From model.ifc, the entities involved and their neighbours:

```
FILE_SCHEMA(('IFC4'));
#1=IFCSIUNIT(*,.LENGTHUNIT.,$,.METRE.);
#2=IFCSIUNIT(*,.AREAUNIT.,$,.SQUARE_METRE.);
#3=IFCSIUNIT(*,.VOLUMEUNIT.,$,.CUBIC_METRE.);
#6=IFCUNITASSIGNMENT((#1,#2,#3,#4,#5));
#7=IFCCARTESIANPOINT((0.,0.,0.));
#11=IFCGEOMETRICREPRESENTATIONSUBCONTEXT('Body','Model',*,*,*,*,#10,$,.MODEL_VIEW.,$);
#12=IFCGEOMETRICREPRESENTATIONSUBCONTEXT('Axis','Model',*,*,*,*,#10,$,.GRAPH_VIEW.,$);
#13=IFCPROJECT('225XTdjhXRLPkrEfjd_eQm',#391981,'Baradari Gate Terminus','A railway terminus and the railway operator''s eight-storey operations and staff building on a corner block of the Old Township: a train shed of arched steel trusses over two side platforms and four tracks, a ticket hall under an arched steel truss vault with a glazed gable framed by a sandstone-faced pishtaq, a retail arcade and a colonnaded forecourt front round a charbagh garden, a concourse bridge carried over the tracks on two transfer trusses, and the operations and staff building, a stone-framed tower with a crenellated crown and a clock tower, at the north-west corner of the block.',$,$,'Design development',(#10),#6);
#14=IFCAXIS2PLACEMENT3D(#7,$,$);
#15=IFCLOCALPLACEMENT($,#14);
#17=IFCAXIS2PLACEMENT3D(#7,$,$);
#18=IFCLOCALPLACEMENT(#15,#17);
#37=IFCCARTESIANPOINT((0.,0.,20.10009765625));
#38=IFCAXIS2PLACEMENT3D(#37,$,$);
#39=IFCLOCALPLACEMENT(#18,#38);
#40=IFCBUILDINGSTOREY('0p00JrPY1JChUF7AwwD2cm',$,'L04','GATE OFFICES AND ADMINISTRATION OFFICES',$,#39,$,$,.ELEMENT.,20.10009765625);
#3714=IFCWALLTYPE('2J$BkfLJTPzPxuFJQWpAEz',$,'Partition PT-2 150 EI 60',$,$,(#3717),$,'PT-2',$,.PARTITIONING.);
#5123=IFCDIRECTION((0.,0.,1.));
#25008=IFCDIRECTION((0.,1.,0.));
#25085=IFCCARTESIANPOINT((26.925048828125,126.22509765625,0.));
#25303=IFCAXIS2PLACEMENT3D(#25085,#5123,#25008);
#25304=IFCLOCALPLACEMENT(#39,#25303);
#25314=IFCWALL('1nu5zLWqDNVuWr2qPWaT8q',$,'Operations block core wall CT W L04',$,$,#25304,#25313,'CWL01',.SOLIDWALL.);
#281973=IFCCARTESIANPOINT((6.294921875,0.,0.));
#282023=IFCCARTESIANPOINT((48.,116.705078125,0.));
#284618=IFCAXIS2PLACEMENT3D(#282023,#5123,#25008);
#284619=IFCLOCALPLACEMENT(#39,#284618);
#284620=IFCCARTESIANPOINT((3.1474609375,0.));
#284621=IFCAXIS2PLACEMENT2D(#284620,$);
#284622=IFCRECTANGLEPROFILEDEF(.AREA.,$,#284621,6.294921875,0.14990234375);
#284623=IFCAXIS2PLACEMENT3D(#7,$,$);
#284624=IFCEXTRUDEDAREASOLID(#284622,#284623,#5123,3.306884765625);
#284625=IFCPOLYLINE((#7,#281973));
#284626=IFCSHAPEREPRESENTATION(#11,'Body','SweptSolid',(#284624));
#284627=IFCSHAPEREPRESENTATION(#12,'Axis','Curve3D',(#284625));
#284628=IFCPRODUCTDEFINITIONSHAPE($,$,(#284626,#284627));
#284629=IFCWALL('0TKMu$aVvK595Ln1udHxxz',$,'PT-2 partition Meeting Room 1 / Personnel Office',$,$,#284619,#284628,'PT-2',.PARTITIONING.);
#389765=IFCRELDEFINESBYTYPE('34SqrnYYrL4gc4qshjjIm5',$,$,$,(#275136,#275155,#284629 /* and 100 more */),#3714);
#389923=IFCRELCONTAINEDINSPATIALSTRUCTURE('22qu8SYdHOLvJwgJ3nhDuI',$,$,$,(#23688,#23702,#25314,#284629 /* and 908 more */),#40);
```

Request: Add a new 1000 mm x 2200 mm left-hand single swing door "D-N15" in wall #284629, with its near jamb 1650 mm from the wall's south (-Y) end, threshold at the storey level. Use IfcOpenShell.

```python
import numpy as np
import ifcopenshell
import ifcopenshell.api.feature
import ifcopenshell.api.geometry
import ifcopenshell.api.root
import ifcopenshell.api.spatial
import ifcopenshell.geom
import ifcopenshell.util.element
import ifcopenshell.util.placement
import ifcopenshell.util.representation
import ifcopenshell.util.shape
import ifcopenshell.util.unit

model = ifcopenshell.open("model.ifc")
unit_scale = ifcopenshell.util.unit.calculate_unit_scale(model)
settings = ifcopenshell.geom.settings()


def volume(element):
    """Net volume in cubic metres, openings subtracted."""
    shape = ifcopenshell.geom.create_shape(settings, element)
    return ifcopenshell.util.shape.get_volume(shape.geometry)


wall = model.by_guid("0TKMu$aVvK595Ln1udHxxz")
storey = ifcopenshell.util.element.get_container(wall, ifc_class="IfcBuildingStorey")
context = ifcopenshell.util.representation.get_context(model, "Model", "Body", "MODEL_VIEW")
before = volume(wall)

width, height, from_end, sill = 1, 2.2, 1.65, 0.0  # metres

# The wall runs along its own X axis, and the end named is its -X end.
wall_shape = ifcopenshell.geom.create_shape(settings, wall)
x, y, z = ifcopenshell.util.shape.get_vertices(wall_shape.geometry).T
start = x.min() + from_end
face, thickness = float(y.min()), float(y.max() - y.min())
wall_matrix = ifcopenshell.util.placement.get_local_placement(wall.ObjectPlacement)
level = ifcopenshell.util.placement.get_local_placement(storey.ObjectPlacement)[2, 3]


def in_wall(x, y):
    """Placement at x, y metres in the wall's axes, at sill height."""
    matrix = wall_matrix.copy()
    matrix[:, 3] = wall_matrix @ np.array([x / unit_scale, y / unit_scale, 0.0, 1.0])
    matrix[2, 3] = level + sill / unit_scale
    return matrix


# Opening: a box that overshoots both wall faces by 50 mm.
opening = ifcopenshell.api.root.create_entity(model, ifc_class="IfcOpeningElement", predefined_type="OPENING")
box = ifcopenshell.api.geometry.add_wall_representation(
    model, context=context, length=width, height=height, thickness=thickness + 0.1
)
ifcopenshell.api.geometry.assign_representation(model, product=opening, representation=box)
ifcopenshell.api.geometry.edit_object_placement(model, product=opening, matrix=in_wall(start, face - 0.05), is_si=False)
ifcopenshell.api.feature.add_feature(model, feature=opening, element=wall)

door = ifcopenshell.api.root.create_entity(model, ifc_class="IfcDoor", name="D-N15", predefined_type="DOOR")
door.OverallWidth, door.OverallHeight = width / unit_scale, height / unit_scale
door.OperationType = "SINGLE_SWING_LEFT"
body = ifcopenshell.api.geometry.add_door_representation(
    model,
    context=context,
    overall_width=door.OverallWidth,
    overall_height=door.OverallHeight,
    operation_type="SINGLE_SWING_LEFT",
    lining_properties={"LiningDepth": thickness / unit_scale, "ThresholdDepth": thickness / unit_scale},
)
ifcopenshell.api.geometry.assign_representation(model, product=door, representation=body)
ifcopenshell.api.spatial.assign_container(model, products=[door], relating_structure=storey)
ifcopenshell.api.feature.add_filling(model, opening=opening, element=door)

# The lining spans the wall, so the door starts at the wall face.
ifcopenshell.api.geometry.edit_object_placement(model, product=door, matrix=in_wall(start, face), is_si=False)

after = volume(wall)

print(f"wall volume {before:.3f} -> {after:.3f} m3")

model.write("model_rev.ifc")
```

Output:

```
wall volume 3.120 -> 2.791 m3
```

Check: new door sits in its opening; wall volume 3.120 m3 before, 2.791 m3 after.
